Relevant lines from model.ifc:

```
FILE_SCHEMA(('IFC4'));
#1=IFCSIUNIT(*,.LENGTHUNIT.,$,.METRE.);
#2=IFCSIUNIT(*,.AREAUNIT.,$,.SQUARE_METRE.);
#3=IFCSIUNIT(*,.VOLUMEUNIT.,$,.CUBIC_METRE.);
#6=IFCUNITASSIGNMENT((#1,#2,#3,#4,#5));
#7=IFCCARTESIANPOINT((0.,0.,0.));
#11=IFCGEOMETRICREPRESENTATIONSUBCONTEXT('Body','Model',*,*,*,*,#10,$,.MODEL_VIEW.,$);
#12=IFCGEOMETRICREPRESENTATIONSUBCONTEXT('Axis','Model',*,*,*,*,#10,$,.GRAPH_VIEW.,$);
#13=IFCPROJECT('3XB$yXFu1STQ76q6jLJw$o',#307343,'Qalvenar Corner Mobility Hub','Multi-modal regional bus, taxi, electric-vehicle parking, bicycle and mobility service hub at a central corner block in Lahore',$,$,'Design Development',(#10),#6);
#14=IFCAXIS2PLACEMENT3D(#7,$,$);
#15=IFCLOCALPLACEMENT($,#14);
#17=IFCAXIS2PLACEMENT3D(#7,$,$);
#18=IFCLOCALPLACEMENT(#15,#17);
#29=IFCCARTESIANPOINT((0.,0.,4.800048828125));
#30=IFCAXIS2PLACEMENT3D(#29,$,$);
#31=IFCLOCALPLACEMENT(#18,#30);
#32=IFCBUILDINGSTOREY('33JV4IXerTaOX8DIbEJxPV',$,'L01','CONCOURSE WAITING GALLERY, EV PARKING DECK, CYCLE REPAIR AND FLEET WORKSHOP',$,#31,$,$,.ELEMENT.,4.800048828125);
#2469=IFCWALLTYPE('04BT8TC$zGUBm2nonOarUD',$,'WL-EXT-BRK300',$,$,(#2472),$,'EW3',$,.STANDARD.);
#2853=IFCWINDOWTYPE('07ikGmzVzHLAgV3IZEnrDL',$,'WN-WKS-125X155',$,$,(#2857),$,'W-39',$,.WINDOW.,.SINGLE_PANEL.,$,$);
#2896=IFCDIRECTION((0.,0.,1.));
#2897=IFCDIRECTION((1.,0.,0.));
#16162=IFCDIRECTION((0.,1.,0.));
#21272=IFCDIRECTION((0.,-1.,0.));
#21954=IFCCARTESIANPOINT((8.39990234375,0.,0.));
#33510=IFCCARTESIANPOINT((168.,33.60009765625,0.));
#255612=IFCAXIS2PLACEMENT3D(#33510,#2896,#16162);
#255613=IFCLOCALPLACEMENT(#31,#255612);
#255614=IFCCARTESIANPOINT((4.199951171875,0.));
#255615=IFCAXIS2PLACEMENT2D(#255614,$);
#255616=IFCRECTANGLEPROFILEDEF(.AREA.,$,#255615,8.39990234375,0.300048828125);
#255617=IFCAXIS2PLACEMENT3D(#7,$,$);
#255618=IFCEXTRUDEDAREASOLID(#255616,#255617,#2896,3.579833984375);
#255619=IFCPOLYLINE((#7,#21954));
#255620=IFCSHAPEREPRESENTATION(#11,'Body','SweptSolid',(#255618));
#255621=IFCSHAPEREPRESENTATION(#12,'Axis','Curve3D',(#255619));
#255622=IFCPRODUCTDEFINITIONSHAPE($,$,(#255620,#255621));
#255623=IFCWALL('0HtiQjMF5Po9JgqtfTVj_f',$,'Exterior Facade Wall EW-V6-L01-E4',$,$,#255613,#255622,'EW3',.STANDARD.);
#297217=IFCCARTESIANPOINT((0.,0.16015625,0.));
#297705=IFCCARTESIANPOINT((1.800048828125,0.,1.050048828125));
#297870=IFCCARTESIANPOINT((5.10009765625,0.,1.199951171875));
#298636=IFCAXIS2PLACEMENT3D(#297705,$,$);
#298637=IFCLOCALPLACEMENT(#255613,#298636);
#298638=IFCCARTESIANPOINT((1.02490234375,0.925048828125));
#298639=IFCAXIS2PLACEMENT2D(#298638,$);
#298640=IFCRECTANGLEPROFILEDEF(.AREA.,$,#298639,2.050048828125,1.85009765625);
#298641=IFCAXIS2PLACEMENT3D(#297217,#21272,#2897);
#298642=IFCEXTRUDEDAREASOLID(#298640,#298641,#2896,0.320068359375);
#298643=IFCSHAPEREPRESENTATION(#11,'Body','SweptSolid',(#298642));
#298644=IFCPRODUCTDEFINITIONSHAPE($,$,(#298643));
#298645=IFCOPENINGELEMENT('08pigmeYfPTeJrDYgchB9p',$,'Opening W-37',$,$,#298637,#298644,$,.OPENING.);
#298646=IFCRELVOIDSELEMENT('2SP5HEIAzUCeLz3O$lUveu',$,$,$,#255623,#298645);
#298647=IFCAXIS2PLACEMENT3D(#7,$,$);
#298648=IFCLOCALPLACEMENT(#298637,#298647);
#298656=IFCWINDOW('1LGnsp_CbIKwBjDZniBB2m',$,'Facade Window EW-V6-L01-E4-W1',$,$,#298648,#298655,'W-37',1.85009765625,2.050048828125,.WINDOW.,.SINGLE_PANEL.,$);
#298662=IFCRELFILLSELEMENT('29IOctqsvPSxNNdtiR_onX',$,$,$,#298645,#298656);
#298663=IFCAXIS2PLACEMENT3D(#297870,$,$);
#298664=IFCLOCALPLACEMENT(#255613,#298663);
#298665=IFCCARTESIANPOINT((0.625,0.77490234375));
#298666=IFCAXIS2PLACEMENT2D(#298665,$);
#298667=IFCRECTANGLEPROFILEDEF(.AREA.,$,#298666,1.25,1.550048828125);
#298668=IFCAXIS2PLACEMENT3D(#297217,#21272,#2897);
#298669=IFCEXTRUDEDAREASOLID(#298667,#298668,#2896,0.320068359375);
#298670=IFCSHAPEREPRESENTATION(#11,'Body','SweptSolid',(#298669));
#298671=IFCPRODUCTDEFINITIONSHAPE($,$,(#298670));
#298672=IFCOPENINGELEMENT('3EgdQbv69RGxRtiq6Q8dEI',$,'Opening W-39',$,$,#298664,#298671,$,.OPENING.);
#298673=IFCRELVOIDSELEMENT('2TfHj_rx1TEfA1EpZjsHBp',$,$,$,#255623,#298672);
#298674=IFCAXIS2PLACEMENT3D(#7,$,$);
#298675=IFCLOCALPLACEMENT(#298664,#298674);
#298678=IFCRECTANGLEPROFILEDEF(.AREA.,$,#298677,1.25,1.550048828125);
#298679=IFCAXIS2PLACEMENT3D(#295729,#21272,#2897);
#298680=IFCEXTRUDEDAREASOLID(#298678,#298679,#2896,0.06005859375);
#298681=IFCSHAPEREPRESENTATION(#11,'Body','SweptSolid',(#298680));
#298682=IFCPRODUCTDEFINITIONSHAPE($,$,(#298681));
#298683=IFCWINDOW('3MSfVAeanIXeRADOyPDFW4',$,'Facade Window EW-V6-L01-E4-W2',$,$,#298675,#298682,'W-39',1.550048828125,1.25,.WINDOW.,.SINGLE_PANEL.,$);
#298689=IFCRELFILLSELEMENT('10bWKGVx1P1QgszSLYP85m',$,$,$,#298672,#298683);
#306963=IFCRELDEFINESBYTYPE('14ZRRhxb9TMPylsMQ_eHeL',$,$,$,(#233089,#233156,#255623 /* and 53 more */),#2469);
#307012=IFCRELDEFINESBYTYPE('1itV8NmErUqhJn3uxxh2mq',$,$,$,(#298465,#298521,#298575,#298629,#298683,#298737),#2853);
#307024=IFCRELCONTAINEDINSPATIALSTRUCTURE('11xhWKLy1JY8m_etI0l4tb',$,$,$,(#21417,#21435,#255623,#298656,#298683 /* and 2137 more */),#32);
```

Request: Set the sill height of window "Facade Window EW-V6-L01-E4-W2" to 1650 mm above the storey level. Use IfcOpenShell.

```python
import numpy as np
import ifcopenshell
import ifcopenshell.api.geometry
import ifcopenshell.geom
import ifcopenshell.util.element
import ifcopenshell.util.placement
import ifcopenshell.util.shape
import ifcopenshell.util.unit

model = ifcopenshell.open("model.ifc")
unit_scale = ifcopenshell.util.unit.calculate_unit_scale(model)

window = model.by_guid("3MSfVAeanIXeRADOyPDFW4")
opening = window.FillsVoids[0].RelatingOpeningElement
storey = ifcopenshell.util.element.get_container(window, ifc_class="IfcBuildingStorey")
level = ifcopenshell.util.placement.get_local_placement(storey.ObjectPlacement)[2, 3]

# The opening's origin need not be at the sill, so measure its lowest point.
shape = ifcopenshell.geom.create_shape(ifcopenshell.geom.settings(), opening)
bottom = ifcopenshell.util.shape.get_shape_bottom_elevation(shape, shape.geometry) / unit_scale
dz = level + 1.65 - bottom

shift = np.array([0.0, 0.0, dz])
# The window is placed relative to its opening, so it follows when the opening moves.
matrix = ifcopenshell.util.placement.get_local_placement(opening.ObjectPlacement)
matrix[:3, 3] += shift
ifcopenshell.api.geometry.edit_object_placement(
    model, product=opening, matrix=matrix, is_si=False, should_transform_children=True
)

print(f"moved by {dz * unit_scale:+.3f} m")

model.write("model_v2.ifc")
```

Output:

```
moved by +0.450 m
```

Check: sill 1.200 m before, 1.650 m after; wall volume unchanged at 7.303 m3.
